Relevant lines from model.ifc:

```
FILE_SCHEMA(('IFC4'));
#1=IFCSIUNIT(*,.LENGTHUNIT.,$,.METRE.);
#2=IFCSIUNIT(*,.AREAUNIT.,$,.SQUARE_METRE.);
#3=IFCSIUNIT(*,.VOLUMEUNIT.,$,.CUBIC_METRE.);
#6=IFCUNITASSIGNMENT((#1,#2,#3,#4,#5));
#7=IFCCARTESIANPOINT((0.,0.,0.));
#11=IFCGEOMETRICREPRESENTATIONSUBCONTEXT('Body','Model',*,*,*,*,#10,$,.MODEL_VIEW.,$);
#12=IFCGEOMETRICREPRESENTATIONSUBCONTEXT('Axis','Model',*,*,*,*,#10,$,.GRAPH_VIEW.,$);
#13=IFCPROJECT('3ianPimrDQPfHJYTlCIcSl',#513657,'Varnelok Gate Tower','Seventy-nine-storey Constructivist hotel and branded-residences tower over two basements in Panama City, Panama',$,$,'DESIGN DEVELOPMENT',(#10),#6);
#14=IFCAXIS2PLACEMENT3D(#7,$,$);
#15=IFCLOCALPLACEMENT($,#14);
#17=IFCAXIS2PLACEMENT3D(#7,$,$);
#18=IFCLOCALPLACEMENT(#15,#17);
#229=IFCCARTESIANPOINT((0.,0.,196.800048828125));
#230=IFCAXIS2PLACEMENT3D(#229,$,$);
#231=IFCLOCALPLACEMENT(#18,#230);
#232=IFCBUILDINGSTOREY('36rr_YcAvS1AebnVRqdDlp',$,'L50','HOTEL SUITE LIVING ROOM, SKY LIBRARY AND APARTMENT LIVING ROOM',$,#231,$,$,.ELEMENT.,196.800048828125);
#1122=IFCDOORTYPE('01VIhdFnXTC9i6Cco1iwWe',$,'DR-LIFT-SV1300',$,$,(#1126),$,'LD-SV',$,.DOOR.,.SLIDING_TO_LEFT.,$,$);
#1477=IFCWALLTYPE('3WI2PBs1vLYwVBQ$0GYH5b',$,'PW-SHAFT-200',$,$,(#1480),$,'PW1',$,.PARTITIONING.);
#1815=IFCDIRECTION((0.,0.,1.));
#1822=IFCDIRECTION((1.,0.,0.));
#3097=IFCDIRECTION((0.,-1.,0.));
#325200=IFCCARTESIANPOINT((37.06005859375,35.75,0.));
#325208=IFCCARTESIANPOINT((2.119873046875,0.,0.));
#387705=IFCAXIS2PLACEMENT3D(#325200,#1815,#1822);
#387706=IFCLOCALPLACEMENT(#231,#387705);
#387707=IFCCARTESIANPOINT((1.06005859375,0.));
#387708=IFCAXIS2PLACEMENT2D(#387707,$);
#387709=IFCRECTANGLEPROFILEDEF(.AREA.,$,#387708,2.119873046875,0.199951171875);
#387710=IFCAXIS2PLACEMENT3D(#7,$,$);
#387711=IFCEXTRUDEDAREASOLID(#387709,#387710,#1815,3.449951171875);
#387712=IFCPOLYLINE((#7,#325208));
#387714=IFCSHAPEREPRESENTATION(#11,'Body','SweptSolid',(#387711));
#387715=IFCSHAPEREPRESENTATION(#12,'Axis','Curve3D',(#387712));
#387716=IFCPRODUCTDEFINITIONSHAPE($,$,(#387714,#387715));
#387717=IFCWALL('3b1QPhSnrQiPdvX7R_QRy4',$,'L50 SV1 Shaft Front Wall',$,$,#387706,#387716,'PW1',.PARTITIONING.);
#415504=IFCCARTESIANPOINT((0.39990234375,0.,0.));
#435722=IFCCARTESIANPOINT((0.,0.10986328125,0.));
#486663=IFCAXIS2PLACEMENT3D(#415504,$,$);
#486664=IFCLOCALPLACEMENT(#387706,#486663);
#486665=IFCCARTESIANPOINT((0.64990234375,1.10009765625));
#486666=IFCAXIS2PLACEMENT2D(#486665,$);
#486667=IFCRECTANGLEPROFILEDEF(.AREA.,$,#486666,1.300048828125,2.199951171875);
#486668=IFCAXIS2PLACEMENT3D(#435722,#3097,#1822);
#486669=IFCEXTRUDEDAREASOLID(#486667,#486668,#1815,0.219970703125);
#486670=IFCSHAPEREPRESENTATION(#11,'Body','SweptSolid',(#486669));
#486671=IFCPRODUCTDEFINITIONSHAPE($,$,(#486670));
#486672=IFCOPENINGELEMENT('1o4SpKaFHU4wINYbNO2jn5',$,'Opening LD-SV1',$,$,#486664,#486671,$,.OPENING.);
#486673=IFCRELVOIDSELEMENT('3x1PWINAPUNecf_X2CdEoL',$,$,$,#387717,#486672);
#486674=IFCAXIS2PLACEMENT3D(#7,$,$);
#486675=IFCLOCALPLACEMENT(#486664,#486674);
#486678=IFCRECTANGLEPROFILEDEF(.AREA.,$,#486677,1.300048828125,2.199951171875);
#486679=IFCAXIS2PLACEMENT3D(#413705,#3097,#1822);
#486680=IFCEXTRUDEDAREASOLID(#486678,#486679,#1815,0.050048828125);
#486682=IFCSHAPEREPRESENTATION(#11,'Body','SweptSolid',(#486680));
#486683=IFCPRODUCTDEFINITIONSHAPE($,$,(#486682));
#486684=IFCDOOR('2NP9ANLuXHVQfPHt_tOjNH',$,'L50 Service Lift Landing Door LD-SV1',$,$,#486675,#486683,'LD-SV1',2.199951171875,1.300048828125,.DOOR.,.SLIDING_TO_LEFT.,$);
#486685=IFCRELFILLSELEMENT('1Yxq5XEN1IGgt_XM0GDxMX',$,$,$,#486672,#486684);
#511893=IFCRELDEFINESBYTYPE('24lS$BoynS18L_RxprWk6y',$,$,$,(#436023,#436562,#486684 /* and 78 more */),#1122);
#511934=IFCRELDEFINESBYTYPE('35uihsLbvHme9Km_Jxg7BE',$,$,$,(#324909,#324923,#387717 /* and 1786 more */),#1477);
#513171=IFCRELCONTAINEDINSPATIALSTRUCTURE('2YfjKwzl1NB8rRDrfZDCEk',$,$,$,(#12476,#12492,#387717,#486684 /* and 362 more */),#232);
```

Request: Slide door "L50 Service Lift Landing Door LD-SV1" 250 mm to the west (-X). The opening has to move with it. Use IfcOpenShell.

```python
import ifcopenshell
import ifcopenshell.api.geometry
import ifcopenshell.util.placement
import ifcopenshell.util.unit

model = ifcopenshell.open("model.ifc")
unit_scale = ifcopenshell.util.unit.calculate_unit_scale(model)

door = model.by_guid("2NP9ANLuXHVQfPHt_tOjNH")
opening = door.FillsVoids[0].RelatingOpeningElement
wall = opening.VoidsElements[0].RelatingBuildingElement

wall_matrix = ifcopenshell.util.placement.get_local_placement(wall.ObjectPlacement)
shift = wall_matrix[:3, 0] * -0.25 / unit_scale
before = ifcopenshell.util.placement.get_local_placement(door.ObjectPlacement)[:3, 3].copy()

# The door is placed relative to its opening, so it follows when the opening moves.
matrix = ifcopenshell.util.placement.get_local_placement(opening.ObjectPlacement)
matrix[:3, 3] += shift
ifcopenshell.api.geometry.edit_object_placement(
    model, product=opening, matrix=matrix, is_si=False, should_transform_children=True
)

after = ifcopenshell.util.placement.get_local_placement(door.ObjectPlacement)[:3, 3]
print("door moved by", (after - before).round(3) + 0.0)

model.write("model_rev.ifc")
```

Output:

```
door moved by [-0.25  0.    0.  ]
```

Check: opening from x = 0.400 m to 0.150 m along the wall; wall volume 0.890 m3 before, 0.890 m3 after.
